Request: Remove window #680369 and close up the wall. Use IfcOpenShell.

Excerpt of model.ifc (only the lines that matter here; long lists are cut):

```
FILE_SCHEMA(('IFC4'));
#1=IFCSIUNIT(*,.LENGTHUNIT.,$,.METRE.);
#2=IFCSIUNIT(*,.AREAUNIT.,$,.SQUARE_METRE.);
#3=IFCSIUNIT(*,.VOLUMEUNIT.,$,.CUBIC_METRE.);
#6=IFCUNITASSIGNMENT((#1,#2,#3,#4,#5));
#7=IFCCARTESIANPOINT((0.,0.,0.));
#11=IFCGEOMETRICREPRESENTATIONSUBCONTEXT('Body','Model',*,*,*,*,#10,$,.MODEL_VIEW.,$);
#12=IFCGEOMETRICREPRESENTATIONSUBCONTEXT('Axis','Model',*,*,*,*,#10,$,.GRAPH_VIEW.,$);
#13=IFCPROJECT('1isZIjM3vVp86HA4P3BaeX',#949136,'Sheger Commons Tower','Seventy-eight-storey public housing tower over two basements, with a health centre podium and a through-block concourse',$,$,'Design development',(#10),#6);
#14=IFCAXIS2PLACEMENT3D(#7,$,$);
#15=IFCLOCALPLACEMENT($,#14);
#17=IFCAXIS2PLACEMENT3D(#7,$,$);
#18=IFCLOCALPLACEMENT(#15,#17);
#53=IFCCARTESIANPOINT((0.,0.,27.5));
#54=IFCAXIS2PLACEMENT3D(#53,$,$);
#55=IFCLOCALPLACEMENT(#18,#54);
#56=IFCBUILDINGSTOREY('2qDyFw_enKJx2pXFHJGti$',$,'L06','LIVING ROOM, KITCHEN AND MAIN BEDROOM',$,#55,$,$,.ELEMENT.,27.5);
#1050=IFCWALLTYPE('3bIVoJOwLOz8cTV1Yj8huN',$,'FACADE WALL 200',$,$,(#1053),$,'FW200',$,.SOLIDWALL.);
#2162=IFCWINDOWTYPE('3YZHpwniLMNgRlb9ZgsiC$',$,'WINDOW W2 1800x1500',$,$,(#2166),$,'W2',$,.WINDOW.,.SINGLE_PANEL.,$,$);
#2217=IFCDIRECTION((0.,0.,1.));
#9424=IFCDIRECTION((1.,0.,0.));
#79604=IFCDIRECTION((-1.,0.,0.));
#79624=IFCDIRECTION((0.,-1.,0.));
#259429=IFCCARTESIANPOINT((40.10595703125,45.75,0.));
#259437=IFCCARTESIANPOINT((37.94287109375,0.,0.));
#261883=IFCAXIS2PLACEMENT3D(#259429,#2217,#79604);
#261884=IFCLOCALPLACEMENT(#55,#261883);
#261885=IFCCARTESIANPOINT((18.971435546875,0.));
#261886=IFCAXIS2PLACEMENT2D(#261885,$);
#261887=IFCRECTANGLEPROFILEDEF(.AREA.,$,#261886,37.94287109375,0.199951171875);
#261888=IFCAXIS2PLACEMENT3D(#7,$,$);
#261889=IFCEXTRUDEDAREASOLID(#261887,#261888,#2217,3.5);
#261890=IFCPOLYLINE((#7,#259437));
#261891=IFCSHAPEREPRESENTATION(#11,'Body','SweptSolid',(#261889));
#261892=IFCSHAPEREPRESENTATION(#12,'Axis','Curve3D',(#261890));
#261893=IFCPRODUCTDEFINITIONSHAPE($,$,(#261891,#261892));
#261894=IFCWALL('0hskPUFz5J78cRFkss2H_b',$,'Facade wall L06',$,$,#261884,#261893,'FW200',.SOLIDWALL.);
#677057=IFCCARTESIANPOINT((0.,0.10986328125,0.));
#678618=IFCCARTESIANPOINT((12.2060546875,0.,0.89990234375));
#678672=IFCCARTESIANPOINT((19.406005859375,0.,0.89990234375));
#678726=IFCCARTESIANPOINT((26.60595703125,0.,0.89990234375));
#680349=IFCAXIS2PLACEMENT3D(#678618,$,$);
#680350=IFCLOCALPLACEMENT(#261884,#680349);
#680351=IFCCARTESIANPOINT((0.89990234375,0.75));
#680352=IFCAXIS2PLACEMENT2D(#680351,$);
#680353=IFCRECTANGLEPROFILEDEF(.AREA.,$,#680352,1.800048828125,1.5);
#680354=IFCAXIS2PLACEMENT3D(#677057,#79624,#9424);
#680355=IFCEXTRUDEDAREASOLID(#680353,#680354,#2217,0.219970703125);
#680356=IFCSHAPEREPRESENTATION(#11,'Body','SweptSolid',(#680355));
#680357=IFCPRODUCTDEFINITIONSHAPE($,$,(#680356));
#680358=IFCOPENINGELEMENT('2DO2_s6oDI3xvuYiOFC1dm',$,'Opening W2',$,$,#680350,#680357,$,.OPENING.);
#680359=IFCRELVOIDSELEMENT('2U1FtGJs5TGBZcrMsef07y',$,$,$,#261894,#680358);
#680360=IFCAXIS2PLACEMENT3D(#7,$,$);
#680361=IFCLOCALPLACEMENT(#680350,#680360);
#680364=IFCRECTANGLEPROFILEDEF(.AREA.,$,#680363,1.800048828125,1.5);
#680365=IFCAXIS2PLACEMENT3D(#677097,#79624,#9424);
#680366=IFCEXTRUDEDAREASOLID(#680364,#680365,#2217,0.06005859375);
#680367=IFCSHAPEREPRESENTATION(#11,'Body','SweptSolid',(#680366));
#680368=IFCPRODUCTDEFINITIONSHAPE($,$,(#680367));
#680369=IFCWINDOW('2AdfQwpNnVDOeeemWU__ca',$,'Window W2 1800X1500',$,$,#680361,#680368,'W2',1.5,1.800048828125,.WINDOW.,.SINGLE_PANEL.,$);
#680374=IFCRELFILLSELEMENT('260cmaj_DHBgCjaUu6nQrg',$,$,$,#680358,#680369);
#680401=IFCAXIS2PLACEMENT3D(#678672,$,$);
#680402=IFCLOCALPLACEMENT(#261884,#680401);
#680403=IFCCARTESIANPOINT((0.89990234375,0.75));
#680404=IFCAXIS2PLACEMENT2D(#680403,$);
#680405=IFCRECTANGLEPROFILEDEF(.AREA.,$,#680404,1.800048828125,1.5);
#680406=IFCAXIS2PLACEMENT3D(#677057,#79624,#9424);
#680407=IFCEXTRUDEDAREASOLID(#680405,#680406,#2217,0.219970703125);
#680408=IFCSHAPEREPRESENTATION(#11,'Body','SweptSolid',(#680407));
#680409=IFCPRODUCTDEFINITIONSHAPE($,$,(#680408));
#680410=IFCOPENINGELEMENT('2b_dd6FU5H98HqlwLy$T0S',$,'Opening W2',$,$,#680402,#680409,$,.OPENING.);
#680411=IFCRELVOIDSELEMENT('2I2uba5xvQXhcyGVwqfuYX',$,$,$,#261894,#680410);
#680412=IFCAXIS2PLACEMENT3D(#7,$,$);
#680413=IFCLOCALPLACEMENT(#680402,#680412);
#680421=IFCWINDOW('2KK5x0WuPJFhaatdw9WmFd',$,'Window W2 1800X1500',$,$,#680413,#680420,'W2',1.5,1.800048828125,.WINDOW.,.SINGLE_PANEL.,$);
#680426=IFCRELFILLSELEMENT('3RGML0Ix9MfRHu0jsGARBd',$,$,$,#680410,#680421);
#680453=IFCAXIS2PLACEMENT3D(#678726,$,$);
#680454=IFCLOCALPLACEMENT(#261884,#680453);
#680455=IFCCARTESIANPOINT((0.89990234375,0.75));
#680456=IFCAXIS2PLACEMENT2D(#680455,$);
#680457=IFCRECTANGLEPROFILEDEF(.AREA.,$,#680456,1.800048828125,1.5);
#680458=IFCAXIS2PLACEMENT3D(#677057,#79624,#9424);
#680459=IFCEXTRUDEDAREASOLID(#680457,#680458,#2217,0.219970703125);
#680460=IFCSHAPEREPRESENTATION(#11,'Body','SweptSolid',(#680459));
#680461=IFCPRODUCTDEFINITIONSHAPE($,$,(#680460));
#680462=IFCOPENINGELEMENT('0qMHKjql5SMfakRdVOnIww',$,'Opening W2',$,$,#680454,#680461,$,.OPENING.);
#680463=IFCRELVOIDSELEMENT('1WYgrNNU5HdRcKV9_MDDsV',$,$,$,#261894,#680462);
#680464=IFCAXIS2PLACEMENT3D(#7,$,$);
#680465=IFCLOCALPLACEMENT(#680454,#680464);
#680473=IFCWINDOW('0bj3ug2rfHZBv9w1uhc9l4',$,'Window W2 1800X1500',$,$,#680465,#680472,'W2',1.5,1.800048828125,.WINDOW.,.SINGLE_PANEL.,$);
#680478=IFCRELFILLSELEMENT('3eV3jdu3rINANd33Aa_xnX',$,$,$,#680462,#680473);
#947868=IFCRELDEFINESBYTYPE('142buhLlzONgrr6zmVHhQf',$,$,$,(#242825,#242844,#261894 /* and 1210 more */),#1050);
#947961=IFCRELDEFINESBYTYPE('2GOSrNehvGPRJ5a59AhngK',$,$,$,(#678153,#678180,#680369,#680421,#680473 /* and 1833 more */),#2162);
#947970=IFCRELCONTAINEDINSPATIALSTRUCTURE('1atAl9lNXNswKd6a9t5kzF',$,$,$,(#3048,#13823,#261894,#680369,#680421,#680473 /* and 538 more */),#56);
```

```python
import ifcopenshell
import ifcopenshell.api.feature
import ifcopenshell.api.root
import ifcopenshell.geom
import ifcopenshell.util.shape

model = ifcopenshell.open("model.ifc")
settings = ifcopenshell.geom.settings()


def volume(element):
    """Net volume in cubic metres, openings subtracted."""
    shape = ifcopenshell.geom.create_shape(settings, element)
    return ifcopenshell.util.shape.get_volume(shape.geometry)


window = model.by_guid("2AdfQwpNnVDOeeemWU__ca")
opening = window.FillsVoids[0].RelatingOpeningElement
wall = opening.VoidsElements[0].RelatingBuildingElement
before = volume(wall)

ifcopenshell.api.root.remove_product(model, product=window)
ifcopenshell.api.feature.remove_feature(model, feature=opening)

after = volume(wall)

print(f"wall volume {before:.3f} -> {after:.3f} m3")

model.write("model-out.ifc")
```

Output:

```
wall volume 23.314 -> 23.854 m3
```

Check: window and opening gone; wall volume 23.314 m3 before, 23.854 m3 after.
